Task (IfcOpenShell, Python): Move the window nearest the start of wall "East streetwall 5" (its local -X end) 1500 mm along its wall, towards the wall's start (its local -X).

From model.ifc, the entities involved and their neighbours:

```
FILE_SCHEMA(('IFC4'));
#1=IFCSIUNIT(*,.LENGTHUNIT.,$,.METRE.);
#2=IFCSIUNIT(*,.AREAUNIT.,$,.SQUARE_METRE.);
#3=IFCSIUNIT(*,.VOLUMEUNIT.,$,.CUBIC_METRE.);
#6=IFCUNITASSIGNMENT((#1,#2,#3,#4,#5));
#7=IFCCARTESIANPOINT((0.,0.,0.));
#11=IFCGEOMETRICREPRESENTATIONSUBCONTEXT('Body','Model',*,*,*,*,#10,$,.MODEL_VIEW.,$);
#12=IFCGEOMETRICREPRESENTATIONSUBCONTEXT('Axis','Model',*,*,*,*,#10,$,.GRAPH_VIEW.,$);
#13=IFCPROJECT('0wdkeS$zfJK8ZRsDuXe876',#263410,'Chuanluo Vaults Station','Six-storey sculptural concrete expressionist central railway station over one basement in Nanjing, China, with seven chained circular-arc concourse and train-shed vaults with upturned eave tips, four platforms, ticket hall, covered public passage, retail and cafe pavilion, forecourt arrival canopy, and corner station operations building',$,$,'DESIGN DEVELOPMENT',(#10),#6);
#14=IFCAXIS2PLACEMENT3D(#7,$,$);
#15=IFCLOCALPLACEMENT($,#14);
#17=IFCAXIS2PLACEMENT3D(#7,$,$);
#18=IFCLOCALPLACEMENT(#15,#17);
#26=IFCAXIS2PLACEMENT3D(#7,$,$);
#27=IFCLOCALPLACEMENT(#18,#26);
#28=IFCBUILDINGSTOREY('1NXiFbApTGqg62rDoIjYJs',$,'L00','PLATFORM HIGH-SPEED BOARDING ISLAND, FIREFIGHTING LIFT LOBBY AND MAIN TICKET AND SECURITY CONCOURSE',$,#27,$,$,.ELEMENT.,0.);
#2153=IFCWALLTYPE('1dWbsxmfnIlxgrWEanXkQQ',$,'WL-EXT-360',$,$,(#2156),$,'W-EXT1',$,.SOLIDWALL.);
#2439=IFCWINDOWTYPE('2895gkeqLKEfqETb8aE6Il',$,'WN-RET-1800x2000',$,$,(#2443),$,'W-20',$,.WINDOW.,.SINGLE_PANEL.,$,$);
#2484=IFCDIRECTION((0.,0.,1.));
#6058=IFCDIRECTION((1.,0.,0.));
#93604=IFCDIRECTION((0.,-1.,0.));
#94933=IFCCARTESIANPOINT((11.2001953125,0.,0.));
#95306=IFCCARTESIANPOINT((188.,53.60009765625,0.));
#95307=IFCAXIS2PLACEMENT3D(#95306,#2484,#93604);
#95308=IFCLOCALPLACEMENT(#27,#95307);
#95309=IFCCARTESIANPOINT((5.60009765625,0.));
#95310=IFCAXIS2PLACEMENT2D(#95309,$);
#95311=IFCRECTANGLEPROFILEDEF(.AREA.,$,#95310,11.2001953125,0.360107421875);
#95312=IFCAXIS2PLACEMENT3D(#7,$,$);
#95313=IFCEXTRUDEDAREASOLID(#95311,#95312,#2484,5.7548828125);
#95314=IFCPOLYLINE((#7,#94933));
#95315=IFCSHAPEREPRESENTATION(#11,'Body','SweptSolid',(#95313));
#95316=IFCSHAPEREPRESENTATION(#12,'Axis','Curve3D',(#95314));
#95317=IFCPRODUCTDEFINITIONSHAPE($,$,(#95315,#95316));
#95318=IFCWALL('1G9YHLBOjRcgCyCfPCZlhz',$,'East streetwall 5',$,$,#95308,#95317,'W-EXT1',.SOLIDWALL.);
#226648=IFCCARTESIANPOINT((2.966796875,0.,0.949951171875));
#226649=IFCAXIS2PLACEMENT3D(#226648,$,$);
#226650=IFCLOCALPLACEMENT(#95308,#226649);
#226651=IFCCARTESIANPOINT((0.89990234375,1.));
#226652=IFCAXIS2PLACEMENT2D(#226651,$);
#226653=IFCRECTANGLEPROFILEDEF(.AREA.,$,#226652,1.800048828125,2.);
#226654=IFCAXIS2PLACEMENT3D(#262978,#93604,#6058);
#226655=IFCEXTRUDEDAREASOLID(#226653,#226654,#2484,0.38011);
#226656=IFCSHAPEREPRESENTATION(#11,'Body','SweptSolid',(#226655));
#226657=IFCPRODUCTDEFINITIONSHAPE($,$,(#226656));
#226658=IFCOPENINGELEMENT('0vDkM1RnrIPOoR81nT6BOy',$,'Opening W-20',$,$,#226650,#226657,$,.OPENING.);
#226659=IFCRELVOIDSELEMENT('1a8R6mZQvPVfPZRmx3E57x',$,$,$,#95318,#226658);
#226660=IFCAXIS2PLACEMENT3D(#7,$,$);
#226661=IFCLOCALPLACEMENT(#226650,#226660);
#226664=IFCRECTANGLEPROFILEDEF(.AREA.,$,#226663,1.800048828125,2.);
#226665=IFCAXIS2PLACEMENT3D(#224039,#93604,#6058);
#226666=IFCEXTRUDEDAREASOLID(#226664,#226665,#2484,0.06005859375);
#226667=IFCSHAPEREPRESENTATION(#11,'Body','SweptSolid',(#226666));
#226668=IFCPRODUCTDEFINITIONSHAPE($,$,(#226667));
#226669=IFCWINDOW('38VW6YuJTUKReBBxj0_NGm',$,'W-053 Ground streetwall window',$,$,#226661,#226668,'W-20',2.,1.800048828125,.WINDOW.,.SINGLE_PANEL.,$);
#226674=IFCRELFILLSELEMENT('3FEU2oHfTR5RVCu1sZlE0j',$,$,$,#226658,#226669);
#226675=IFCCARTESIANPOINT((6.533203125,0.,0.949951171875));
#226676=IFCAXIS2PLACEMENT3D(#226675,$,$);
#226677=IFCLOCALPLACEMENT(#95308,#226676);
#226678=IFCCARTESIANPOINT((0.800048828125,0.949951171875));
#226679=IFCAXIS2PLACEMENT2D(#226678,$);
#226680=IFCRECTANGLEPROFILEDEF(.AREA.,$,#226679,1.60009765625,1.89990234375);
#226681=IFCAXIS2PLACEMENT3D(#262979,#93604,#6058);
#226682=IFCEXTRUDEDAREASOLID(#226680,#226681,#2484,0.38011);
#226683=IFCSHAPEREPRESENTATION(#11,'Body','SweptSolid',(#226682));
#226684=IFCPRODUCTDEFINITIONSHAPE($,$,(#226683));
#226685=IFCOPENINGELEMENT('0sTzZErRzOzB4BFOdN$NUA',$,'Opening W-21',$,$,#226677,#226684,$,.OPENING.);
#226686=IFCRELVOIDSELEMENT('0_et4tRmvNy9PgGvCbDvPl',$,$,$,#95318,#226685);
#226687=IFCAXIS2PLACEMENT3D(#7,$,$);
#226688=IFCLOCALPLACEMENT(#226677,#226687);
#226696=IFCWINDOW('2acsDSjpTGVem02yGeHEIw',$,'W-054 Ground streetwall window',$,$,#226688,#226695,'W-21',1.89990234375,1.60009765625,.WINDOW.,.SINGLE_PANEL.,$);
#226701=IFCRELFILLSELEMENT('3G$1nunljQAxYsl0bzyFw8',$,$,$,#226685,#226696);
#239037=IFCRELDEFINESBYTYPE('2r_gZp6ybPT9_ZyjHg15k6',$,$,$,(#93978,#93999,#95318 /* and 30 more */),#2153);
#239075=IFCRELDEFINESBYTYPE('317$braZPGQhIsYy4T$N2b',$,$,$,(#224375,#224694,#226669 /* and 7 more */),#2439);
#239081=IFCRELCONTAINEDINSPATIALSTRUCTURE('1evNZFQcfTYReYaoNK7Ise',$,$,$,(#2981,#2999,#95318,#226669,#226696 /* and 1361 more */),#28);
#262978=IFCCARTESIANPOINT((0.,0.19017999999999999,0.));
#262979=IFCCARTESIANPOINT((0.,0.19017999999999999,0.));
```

```python
import ifcopenshell
import ifcopenshell.api.geometry
import ifcopenshell.util.placement

model = ifcopenshell.open("model.ifc")

window = model.by_guid("38VW6YuJTUKReBBxj0_NGm")
opening = window.FillsVoids[0].RelatingOpeningElement
wall = opening.VoidsElements[0].RelatingBuildingElement

wall_matrix = ifcopenshell.util.placement.get_local_placement(wall.ObjectPlacement)
shift = wall_matrix[:3, 0] * -1.5
before = ifcopenshell.util.placement.get_local_placement(window.ObjectPlacement)[:3, 3].copy()

# The window is placed relative to its opening, so it follows when the opening moves.
matrix = ifcopenshell.util.placement.get_local_placement(opening.ObjectPlacement)
matrix[:3, 3] += shift
ifcopenshell.api.geometry.edit_object_placement(
    model, product=opening, matrix=matrix, is_si=False, should_transform_children=True
)

after = ifcopenshell.util.placement.get_local_placement(window.ObjectPlacement)[:3, 3]
print("window moved by", (after - before).round(3) + 0.0)

model.write("model_edited.ifc")
```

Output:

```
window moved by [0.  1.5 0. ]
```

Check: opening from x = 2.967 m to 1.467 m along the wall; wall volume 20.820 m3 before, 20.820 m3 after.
